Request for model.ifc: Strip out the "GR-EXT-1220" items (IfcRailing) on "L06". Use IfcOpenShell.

First a look at what the model holds.

```python
import ifcopenshell
import ifcopenshell.util.element

model = ifcopenshell.open("model.ifc")
print(model.schema)
storey = next(s for s in model.by_type("IfcBuildingStorey") if s.Name == "L06")
railings = [e for e in ifcopenshell.util.element.get_decomposition(storey) if e.is_a("IfcRailing")]
seen = {}
for e in railings:
    element_type = ifcopenshell.util.element.get_type(e)
    name = element_type.Name if element_type not in (None, e) else None
    seen[name] = seen.get(name, 0) + 1
for name, count in sorted(seen.items(), key=str):
    print(count, "x", name)
```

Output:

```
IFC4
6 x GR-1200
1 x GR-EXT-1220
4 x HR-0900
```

```python
import ifcopenshell
import ifcopenshell.api.root
import ifcopenshell.util.element

model = ifcopenshell.open("model.ifc")

storey = next(s for s in model.by_type("IfcBuildingStorey") if s.Name == "L06")
railings = [e for e in ifcopenshell.util.element.get_decomposition(storey) if e.is_a("IfcRailing")]
targets = [e for e in railings if (t := ifcopenshell.util.element.get_type(e)) not in (None, e) and t.Name == "GR-EXT-1220"]

for e in targets:
    ifcopenshell.api.root.remove_product(model, product=e)
print(len(targets), "removed")

model.write("model_edited.ifc")
```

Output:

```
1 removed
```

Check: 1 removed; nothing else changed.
